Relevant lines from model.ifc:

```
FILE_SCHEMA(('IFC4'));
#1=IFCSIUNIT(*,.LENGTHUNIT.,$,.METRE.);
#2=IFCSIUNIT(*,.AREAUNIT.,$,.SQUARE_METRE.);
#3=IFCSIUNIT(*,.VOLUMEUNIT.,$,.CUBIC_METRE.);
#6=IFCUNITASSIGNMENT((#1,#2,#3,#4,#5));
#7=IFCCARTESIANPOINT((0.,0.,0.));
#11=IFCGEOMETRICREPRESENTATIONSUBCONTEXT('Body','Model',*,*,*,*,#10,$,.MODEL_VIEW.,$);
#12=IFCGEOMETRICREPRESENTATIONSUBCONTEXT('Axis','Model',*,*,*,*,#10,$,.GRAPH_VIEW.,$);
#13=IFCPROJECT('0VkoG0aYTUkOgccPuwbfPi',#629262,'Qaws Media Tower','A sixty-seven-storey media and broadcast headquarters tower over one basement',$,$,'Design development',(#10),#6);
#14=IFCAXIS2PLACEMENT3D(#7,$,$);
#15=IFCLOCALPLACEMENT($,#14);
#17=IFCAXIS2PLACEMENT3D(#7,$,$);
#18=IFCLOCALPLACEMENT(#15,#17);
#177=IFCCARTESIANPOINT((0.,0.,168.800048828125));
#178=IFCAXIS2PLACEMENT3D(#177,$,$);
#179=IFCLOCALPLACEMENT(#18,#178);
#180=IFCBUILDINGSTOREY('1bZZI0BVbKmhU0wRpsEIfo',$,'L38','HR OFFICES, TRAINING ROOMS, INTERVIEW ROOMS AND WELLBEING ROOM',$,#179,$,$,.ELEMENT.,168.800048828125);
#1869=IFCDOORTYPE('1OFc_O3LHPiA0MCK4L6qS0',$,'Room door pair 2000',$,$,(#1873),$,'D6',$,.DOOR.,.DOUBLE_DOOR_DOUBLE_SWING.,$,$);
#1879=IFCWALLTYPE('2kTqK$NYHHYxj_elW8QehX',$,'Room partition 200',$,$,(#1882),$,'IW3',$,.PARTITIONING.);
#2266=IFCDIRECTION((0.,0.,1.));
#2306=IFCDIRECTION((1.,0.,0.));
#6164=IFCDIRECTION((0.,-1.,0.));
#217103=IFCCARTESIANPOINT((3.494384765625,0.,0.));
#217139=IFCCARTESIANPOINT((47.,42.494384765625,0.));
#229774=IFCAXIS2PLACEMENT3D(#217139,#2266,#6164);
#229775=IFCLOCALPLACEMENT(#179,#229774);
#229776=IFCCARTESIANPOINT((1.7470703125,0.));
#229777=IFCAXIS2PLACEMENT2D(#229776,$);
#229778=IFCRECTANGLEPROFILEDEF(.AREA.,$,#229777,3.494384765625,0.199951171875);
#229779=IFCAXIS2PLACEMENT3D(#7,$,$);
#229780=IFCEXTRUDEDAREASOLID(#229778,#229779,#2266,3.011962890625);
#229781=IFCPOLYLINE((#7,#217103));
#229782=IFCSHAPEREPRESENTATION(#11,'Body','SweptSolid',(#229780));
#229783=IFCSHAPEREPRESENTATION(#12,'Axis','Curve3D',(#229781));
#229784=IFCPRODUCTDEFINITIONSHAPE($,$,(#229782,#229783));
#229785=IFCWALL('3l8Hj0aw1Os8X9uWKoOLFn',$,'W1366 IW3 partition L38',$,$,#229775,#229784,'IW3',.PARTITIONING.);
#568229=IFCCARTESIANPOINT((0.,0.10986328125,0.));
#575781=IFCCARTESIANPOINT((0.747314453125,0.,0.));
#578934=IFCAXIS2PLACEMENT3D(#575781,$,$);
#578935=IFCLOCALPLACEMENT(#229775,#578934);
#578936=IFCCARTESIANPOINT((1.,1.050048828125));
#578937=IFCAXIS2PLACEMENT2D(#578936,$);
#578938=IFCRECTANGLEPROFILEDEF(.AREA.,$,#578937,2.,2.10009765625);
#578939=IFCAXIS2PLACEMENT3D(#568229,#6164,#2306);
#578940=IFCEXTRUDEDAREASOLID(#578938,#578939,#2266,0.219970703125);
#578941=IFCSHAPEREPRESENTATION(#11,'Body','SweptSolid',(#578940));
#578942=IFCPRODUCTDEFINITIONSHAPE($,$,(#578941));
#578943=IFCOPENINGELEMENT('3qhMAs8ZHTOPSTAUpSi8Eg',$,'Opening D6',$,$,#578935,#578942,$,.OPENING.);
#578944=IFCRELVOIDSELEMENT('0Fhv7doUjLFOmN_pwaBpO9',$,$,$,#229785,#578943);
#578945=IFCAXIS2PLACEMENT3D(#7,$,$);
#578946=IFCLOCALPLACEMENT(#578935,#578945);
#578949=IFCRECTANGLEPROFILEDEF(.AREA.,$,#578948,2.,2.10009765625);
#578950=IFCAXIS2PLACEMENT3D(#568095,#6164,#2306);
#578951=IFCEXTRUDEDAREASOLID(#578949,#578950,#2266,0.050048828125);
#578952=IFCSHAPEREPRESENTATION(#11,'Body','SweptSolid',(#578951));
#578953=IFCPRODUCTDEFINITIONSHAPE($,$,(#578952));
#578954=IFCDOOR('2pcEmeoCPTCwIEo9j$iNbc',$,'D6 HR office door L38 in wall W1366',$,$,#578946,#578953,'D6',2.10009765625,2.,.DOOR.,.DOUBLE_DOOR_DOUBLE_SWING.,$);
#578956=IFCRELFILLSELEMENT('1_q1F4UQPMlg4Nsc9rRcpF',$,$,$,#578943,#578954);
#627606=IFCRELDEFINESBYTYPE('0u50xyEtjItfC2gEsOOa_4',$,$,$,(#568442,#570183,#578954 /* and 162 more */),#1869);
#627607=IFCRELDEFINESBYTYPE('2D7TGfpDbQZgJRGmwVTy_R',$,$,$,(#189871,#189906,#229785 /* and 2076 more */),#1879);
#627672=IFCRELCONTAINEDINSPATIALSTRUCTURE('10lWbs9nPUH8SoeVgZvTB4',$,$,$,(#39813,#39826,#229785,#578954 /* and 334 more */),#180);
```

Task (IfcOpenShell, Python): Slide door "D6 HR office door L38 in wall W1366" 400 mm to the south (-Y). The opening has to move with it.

```python
import ifcopenshell
import ifcopenshell.api.geometry
import ifcopenshell.util.placement
import ifcopenshell.util.unit

model = ifcopenshell.open("model.ifc")
unit_scale = ifcopenshell.util.unit.calculate_unit_scale(model)

door = model.by_guid("2pcEmeoCPTCwIEo9j$iNbc")
opening = door.FillsVoids[0].RelatingOpeningElement
wall = opening.VoidsElements[0].RelatingBuildingElement

wall_matrix = ifcopenshell.util.placement.get_local_placement(wall.ObjectPlacement)
shift = wall_matrix[:3, 0] * 0.4 / unit_scale
before = ifcopenshell.util.placement.get_local_placement(door.ObjectPlacement)[:3, 3].copy()

# The door is placed relative to its opening, so it follows when the opening moves.
matrix = ifcopenshell.util.placement.get_local_placement(opening.ObjectPlacement)
matrix[:3, 3] += shift
ifcopenshell.api.geometry.edit_object_placement(
    model, product=opening, matrix=matrix, is_si=False, should_transform_children=True
)

after = ifcopenshell.util.placement.get_local_placement(door.ObjectPlacement)[:3, 3]
print("door moved by", (after - before).round(3) + 0.0)

model.write("model-out.ifc")
```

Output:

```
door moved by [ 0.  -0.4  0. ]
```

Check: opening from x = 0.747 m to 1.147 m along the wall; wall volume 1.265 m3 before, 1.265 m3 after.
